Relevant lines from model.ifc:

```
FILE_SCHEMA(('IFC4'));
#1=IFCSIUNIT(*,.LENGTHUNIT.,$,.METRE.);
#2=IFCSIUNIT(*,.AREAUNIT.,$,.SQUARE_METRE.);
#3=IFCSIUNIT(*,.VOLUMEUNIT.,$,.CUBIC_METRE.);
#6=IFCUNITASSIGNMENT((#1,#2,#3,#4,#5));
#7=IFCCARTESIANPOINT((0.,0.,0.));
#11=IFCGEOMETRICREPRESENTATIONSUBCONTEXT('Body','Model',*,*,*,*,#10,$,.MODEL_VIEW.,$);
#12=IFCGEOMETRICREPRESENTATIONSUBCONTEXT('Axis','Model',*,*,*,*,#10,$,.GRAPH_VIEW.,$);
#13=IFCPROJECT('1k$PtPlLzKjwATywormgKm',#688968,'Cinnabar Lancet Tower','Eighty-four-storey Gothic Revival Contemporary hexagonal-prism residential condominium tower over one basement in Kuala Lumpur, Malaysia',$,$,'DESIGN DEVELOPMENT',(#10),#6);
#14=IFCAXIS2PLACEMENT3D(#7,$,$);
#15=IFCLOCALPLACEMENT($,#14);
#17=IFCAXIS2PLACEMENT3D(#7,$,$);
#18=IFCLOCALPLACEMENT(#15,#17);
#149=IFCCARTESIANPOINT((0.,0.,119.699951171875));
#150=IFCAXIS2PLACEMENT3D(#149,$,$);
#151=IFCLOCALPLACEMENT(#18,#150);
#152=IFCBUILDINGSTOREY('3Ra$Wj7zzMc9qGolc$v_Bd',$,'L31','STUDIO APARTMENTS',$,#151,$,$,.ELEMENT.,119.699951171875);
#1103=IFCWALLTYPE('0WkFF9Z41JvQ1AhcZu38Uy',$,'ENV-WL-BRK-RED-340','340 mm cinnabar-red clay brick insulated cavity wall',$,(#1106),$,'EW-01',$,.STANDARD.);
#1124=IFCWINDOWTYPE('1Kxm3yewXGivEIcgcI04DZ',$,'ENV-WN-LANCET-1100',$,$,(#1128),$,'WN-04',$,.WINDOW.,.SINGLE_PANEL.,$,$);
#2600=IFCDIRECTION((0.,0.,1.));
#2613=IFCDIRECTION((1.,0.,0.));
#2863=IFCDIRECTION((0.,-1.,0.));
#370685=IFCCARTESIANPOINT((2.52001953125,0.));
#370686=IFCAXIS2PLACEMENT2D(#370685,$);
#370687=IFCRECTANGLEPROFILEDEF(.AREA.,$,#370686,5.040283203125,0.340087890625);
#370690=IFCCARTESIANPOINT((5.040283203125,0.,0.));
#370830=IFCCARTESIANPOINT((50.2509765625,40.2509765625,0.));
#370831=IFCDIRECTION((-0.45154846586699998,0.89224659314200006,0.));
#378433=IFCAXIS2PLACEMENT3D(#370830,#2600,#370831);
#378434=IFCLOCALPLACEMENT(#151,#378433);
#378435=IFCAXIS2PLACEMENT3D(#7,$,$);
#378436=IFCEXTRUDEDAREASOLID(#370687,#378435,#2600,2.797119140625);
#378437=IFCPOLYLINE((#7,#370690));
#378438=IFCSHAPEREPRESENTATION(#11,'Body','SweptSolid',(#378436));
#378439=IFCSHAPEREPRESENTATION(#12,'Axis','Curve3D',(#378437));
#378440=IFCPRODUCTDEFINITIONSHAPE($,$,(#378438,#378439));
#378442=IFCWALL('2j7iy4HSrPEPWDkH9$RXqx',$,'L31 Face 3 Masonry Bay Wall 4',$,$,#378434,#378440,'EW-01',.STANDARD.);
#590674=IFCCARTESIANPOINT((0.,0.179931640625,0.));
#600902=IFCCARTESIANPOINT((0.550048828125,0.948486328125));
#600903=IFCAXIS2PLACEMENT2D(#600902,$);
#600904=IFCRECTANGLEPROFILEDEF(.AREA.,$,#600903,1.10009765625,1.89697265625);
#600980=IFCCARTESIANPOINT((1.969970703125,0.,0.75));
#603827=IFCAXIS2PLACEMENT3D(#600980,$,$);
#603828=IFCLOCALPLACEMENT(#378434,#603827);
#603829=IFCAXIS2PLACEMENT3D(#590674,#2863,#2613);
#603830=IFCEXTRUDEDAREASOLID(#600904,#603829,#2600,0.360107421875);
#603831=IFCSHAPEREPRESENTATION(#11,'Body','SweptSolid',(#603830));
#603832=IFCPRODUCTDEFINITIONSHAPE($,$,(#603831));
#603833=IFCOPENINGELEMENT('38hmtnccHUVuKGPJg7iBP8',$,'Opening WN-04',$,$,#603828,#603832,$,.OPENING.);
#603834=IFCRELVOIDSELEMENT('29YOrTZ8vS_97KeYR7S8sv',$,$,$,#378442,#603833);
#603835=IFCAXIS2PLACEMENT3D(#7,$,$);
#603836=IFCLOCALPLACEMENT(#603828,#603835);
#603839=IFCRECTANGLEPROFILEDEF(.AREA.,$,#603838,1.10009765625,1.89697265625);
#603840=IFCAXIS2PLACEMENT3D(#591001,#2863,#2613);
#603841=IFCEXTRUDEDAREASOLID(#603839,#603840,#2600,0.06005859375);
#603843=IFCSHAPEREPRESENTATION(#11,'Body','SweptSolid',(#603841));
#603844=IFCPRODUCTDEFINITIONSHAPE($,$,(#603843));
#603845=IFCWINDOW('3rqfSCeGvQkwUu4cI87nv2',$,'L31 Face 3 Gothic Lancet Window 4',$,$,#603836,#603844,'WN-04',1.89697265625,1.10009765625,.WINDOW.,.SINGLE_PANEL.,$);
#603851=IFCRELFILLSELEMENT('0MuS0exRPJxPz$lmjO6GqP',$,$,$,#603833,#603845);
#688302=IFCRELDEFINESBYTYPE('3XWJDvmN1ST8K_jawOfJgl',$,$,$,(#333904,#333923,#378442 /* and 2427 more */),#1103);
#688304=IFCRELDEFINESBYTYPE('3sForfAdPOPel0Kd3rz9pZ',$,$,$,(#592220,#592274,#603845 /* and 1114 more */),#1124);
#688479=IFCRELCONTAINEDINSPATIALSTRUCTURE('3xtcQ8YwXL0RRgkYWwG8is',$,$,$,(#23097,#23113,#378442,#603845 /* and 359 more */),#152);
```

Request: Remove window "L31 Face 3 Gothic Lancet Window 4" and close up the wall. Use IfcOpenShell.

```python
import ifcopenshell
import ifcopenshell.api.feature
import ifcopenshell.api.root
import ifcopenshell.geom
import ifcopenshell.util.shape

model = ifcopenshell.open("model.ifc")
settings = ifcopenshell.geom.settings()


def volume(element):
    """Net volume in cubic metres, openings subtracted."""
    shape = ifcopenshell.geom.create_shape(settings, element)
    return ifcopenshell.util.shape.get_volume(shape.geometry)


window = model.by_id(603845)
opening = window.FillsVoids[0].RelatingOpeningElement
wall = opening.VoidsElements[0].RelatingBuildingElement
before = volume(wall)

ifcopenshell.api.root.remove_product(model, product=window)
ifcopenshell.api.feature.remove_feature(model, feature=opening)

after = volume(wall)

print(f"wall volume {before:.3f} -> {after:.3f} m3")

model.write("model_edited.ifc")
```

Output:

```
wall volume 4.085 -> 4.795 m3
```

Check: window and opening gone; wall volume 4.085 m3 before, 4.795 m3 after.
